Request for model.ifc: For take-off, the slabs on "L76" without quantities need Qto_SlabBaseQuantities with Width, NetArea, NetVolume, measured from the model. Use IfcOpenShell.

First a look at what the model holds.

```python
import ifcopenshell
import ifcopenshell.util.element
import ifcopenshell.util.unit

model = ifcopenshell.open("model.ifc")
print(model.schema)
for unit_type in ("LENGTHUNIT", "AREAUNIT", "VOLUMEUNIT"):
    print(unit_type, ifcopenshell.util.unit.calculate_unit_scale(model, unit_type))
storey = next(s for s in model.by_type("IfcBuildingStorey") if s.Name == "L76")
slabs = [e for e in ifcopenshell.util.element.get_decomposition(storey) if e.is_a("IfcSlab")]
for e in sorted(slabs, key=lambda e: e.id()):
    print(e.id(), e.is_a(), e.Name, list(ifcopenshell.util.element.get_psets(e, qtos_only=True)), sep=" | ")
```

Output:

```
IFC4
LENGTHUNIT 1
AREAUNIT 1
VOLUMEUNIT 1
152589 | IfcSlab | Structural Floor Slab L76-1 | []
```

```python
import ifcopenshell
import ifcopenshell.api.pset
import ifcopenshell.geom
import ifcopenshell.util.element
import ifcopenshell.util.shape
import ifcopenshell.util.unit

model = ifcopenshell.open("model.ifc")
unit_scale = ifcopenshell.util.unit.calculate_unit_scale(model)
area_scale = ifcopenshell.util.unit.calculate_unit_scale(model, "AREAUNIT")
volume_scale = ifcopenshell.util.unit.calculate_unit_scale(model, "VOLUMEUNIT")
settings = ifcopenshell.geom.settings()

storey = next(s for s in model.by_type("IfcBuildingStorey") if s.Name == "L76")
slabs = [e for e in ifcopenshell.util.element.get_decomposition(storey) if e.is_a("IfcSlab")]

for e in sorted(slabs, key=lambda e: e.id()):
    if ifcopenshell.util.element.get_psets(e, qtos_only=True, should_inherit=False):
        continue
    # Geometry comes back in metres, in the element's own axes.
    shape = ifcopenshell.geom.create_shape(settings, e)
    values = {
        "Width": ifcopenshell.util.shape.get_z(shape.geometry) / unit_scale,
        "NetArea": ifcopenshell.util.shape.get_footprint_area(shape.geometry) / area_scale,
        "NetVolume": ifcopenshell.util.shape.get_volume(shape.geometry) / volume_scale,
    }
    qto = ifcopenshell.api.pset.add_qto(model, product=e, name="Qto_SlabBaseQuantities")
    ifcopenshell.api.pset.edit_qto(model, qto=qto, properties=values)
    print(e.id(), {k: round(v, 3) for k, v in values.items()})

model.write("model_rev.ifc")
```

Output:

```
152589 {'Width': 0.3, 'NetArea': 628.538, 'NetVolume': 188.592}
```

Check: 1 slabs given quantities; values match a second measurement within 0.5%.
